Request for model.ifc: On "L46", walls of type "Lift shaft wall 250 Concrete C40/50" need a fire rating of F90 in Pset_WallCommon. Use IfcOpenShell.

First a look at what the model holds.

```python
import ifcopenshell
import ifcopenshell.util.element

model = ifcopenshell.open("model.ifc")
print(model.schema)
storey = next(s for s in model.by_type("IfcBuildingStorey") if s.Name == "L46")
walls = [e for e in ifcopenshell.util.element.get_decomposition(storey) if e.is_a("IfcWall")]
seen = {}
for e in walls:
    element_type = ifcopenshell.util.element.get_type(e)
    key = (element_type.Name if element_type != e and element_type else None, ifcopenshell.util.element.get_pset(e, "Pset_WallCommon", "FireRating"))
    seen[key] = seen.get(key, 0) + 1
for (name, value), count in sorted(seen.items(), key=str):
    print(count, "x", name, "|", value)
```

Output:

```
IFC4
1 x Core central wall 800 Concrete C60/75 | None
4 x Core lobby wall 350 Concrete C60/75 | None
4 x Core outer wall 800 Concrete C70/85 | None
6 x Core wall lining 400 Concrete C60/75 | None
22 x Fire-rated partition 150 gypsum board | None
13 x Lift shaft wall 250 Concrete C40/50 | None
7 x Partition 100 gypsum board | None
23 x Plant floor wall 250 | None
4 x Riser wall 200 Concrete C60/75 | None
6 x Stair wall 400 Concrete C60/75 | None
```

```python
import ifcopenshell
import ifcopenshell.api.pset
import ifcopenshell.util.element

model = ifcopenshell.open("model.ifc")

storey = next(s for s in model.by_type("IfcBuildingStorey") if s.Name == "L46")
walls = [e for e in ifcopenshell.util.element.get_decomposition(storey) if e.is_a("IfcWall")]

count = 0
for e in walls:
    element_type = ifcopenshell.util.element.get_type(e)
    if element_type in (None, e) or element_type.Name != "Lift shaft wall 250 Concrete C40/50":
        continue
    found = ifcopenshell.util.element.get_pset(e, "Pset_WallCommon", should_inherit=False)
    if found:
        pset = model.by_id(found["id"])
        if len(ifcopenshell.util.element.get_elements_by_pset(pset)) > 1:
            pset = ifcopenshell.api.pset.unshare_pset(model, products=[e], pset=pset)[0]
    else:
        pset = ifcopenshell.api.pset.add_pset(model, product=e, name="Pset_WallCommon")
    ifcopenshell.api.pset.edit_pset(model, pset=pset, properties={"FireRating": "F90"})
    count += 1

print(count, "walls updated")

model.write("model_rev.ifc")
```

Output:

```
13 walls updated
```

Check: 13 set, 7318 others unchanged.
